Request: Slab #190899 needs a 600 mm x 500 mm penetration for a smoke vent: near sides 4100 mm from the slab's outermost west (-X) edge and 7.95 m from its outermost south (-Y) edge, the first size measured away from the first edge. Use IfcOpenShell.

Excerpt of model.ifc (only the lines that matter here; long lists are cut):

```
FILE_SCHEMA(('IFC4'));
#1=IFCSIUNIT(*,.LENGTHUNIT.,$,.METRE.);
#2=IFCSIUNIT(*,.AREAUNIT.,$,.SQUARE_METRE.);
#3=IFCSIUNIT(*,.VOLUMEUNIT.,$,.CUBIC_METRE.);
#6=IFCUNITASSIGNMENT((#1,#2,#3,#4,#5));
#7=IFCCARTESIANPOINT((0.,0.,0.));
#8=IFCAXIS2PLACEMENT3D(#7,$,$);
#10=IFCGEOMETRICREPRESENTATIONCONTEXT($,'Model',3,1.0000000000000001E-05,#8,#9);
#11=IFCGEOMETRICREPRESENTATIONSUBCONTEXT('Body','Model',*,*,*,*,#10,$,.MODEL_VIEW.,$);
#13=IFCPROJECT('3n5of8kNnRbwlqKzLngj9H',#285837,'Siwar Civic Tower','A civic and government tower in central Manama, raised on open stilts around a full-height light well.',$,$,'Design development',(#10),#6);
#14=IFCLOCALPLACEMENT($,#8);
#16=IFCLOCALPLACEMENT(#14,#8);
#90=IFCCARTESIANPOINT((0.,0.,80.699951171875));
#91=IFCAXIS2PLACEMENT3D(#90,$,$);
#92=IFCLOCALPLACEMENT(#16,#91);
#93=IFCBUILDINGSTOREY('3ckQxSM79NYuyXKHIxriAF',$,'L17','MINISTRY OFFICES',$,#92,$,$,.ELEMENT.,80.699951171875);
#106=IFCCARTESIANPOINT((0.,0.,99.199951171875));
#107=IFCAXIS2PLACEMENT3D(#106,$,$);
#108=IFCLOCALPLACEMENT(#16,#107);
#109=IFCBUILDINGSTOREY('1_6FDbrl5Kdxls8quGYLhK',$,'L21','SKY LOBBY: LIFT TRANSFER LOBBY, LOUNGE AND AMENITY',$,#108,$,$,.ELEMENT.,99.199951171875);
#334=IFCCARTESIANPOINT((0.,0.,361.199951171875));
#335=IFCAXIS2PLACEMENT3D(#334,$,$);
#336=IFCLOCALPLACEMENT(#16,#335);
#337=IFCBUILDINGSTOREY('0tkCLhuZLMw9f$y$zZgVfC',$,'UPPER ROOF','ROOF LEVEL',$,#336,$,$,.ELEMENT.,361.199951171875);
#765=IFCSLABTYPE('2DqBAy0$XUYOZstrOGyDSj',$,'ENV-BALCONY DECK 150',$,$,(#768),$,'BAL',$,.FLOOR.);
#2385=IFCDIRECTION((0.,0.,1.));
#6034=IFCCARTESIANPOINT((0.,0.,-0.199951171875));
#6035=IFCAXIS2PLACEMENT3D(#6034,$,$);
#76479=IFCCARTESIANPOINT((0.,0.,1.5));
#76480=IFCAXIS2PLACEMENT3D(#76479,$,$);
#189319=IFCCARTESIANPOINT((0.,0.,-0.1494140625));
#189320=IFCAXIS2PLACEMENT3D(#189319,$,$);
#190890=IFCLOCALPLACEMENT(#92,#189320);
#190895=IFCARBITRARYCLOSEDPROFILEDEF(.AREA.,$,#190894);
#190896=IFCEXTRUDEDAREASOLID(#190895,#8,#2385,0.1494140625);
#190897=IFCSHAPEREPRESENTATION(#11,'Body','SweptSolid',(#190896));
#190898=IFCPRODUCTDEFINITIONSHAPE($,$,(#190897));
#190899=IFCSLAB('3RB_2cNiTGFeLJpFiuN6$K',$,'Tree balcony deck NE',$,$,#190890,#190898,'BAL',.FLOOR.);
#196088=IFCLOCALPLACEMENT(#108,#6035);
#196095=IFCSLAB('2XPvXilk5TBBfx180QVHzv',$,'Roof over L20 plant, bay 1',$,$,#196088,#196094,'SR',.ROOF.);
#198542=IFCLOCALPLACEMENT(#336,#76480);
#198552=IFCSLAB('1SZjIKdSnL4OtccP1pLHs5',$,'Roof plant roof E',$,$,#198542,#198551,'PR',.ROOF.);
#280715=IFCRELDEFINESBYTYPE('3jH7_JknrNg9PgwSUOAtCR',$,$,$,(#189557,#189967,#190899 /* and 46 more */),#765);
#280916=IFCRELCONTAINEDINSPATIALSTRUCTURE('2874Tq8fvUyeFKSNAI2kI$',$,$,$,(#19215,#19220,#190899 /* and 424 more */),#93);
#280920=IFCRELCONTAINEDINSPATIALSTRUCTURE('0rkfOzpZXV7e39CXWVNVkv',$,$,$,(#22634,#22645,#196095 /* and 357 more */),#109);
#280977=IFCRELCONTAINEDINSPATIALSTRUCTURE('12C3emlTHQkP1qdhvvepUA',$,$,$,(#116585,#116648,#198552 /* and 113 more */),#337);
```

```python
import numpy as np
import ifcopenshell
import ifcopenshell.api.feature
import ifcopenshell.api.geometry
import ifcopenshell.api.root
import ifcopenshell.geom
import ifcopenshell.util.placement
import ifcopenshell.util.representation
import ifcopenshell.util.shape
import ifcopenshell.util.unit

model = ifcopenshell.open("model.ifc")
unit_scale = ifcopenshell.util.unit.calculate_unit_scale(model)
settings = ifcopenshell.geom.settings()


def volume(element):
    """Net volume in cubic metres, openings subtracted."""
    shape = ifcopenshell.geom.create_shape(settings, element)
    return ifcopenshell.util.shape.get_volume(shape.geometry)


slab = model.by_guid("3RB_2cNiTGFeLJpFiuN6$K")
before = volume(slab)

# Extent in the slab's own axes, in metres. The edges named are its -X and -Y sides.
slab_shape = ifcopenshell.geom.create_shape(settings, slab)
vertices = ifcopenshell.util.shape.get_vertices(slab_shape.geometry)
x_min, y_min, bottom = vertices.min(axis=0)
top = vertices[:, 2].max()

opening = ifcopenshell.api.root.create_entity(model, ifc_class="IfcOpeningElement", name="Smoke vent opening", predefined_type="OPENING")
context = ifcopenshell.util.representation.get_context(model, "Model", "Body", "MODEL_VIEW")
width, depth = 0.6, 0.5
outline = [(0.0, 0.0), (width, 0.0), (width, depth), (0.0, depth), (0.0, 0.0)]
# Overshoot both faces by 50 mm so the cut is clean.
shape = ifcopenshell.api.geometry.add_slab_representation(
    model, context=context, depth=top - bottom + 0.1, polyline=outline
)
ifcopenshell.api.geometry.assign_representation(model, product=opening, representation=shape)

matrix = ifcopenshell.util.placement.get_local_placement(slab.ObjectPlacement)
matrix[:, 3] = matrix @ np.append(np.array([x_min + 4.1, y_min + 7.95, bottom - 0.05]) / unit_scale, 1.0)
ifcopenshell.api.geometry.edit_object_placement(model, product=opening, matrix=matrix, is_si=False)
ifcopenshell.api.feature.add_feature(model, feature=opening, element=slab)

after = volume(slab)

print(f"slab volume {before:.3f} -> {after:.3f} m3")

model.write("model_edited.ifc")
```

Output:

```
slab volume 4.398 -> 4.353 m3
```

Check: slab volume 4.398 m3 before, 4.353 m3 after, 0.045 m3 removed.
